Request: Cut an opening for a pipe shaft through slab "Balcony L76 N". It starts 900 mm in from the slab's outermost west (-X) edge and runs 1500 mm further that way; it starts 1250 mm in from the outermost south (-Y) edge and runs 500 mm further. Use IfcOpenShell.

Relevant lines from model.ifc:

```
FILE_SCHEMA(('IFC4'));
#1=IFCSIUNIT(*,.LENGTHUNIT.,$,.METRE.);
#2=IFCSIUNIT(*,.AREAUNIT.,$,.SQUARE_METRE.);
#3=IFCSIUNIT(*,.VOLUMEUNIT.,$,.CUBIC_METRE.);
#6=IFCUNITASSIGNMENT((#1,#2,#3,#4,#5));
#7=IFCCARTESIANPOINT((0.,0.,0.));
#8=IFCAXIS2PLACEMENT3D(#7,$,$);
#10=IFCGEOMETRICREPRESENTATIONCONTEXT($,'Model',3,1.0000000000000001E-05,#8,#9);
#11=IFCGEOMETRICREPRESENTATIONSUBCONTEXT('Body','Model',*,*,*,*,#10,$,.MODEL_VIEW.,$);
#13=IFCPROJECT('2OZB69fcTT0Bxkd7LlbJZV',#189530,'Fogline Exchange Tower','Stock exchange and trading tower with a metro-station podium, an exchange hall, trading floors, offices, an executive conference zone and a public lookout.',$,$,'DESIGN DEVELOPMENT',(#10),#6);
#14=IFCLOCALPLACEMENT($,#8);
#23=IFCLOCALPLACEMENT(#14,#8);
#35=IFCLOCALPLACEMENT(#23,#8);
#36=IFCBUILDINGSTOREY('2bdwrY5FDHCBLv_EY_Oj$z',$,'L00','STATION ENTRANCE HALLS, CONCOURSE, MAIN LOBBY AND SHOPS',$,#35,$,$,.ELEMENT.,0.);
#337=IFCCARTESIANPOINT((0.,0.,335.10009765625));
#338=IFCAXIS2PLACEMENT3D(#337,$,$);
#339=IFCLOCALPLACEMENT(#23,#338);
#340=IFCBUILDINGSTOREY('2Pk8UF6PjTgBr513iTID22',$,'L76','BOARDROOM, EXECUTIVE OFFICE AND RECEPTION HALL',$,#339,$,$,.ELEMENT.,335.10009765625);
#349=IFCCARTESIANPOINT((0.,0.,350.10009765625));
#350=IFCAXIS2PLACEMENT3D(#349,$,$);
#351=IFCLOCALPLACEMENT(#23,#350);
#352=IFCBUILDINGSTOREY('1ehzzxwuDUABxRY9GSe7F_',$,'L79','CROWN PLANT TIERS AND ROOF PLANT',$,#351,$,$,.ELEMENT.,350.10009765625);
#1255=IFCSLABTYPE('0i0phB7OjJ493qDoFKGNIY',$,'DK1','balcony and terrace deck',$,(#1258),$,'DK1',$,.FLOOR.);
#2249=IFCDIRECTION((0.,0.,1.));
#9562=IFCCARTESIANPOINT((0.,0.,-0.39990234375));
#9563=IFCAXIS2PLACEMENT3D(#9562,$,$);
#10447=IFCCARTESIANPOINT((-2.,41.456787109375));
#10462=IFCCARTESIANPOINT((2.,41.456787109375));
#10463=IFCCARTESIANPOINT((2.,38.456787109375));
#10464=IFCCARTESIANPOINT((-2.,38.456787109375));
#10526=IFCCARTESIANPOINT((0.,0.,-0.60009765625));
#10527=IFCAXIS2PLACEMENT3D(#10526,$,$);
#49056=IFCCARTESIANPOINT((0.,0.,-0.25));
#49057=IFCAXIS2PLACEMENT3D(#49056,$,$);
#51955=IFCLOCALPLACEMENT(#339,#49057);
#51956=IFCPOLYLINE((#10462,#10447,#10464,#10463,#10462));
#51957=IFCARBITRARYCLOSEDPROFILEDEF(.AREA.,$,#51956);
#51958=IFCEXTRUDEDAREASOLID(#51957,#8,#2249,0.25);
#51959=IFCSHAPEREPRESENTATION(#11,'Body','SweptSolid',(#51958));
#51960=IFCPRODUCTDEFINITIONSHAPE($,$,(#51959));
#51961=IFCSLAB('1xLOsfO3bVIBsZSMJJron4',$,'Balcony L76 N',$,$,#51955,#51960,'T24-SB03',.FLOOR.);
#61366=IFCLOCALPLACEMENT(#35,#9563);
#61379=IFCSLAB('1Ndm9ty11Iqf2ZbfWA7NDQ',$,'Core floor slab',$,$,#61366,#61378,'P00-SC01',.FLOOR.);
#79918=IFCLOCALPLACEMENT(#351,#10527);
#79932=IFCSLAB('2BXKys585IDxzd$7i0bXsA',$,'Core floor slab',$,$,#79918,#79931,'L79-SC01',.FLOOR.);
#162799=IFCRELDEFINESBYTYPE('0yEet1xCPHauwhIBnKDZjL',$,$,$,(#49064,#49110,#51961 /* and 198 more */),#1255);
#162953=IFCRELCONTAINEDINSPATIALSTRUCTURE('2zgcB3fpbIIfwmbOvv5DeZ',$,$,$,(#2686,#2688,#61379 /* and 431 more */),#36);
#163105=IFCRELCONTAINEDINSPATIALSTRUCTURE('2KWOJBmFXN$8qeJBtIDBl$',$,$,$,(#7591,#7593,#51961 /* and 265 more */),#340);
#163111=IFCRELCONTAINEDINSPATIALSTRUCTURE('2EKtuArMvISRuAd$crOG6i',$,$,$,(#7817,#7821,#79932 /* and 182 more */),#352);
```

```python
import numpy as np
import ifcopenshell
import ifcopenshell.api.feature
import ifcopenshell.api.geometry
import ifcopenshell.api.root
import ifcopenshell.geom
import ifcopenshell.util.placement
import ifcopenshell.util.representation
import ifcopenshell.util.shape
import ifcopenshell.util.unit

model = ifcopenshell.open("model.ifc")
unit_scale = ifcopenshell.util.unit.calculate_unit_scale(model)
settings = ifcopenshell.geom.settings()


def volume(element):
    """Net volume in cubic metres, openings subtracted."""
    shape = ifcopenshell.geom.create_shape(settings, element)
    return ifcopenshell.util.shape.get_volume(shape.geometry)


slab = model.by_guid("1xLOsfO3bVIBsZSMJJron4")
before = volume(slab)

# Extent in the slab's own axes, in metres. The edges named are its -X and -Y sides.
slab_shape = ifcopenshell.geom.create_shape(settings, slab)
vertices = ifcopenshell.util.shape.get_vertices(slab_shape.geometry)
x_min, y_min, bottom = vertices.min(axis=0)
top = vertices[:, 2].max()

opening = ifcopenshell.api.root.create_entity(model, ifc_class="IfcOpeningElement", name="Pipe shaft opening", predefined_type="OPENING")
context = ifcopenshell.util.representation.get_context(model, "Model", "Body", "MODEL_VIEW")
width, depth = 1.5, 0.5
outline = [(0.0, 0.0), (width, 0.0), (width, depth), (0.0, depth), (0.0, 0.0)]
# Overshoot both faces by 50 mm so the cut is clean.
shape = ifcopenshell.api.geometry.add_slab_representation(
    model, context=context, depth=top - bottom + 0.1, polyline=outline
)
ifcopenshell.api.geometry.assign_representation(model, product=opening, representation=shape)

matrix = ifcopenshell.util.placement.get_local_placement(slab.ObjectPlacement)
matrix[:, 3] = matrix @ np.append(np.array([x_min + 0.9, y_min + 1.25, bottom - 0.05]) / unit_scale, 1.0)
ifcopenshell.api.geometry.edit_object_placement(model, product=opening, matrix=matrix, is_si=False)
ifcopenshell.api.feature.add_feature(model, feature=opening, element=slab)

after = volume(slab)

print(f"slab volume {before:.3f} -> {after:.3f} m3")

model.write("model_updated.ifc")
```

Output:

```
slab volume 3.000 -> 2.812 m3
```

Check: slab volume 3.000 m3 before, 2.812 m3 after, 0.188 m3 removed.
